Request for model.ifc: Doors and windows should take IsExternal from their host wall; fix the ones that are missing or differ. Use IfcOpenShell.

First a look at what the model holds.

```python
import ifcopenshell
import ifcopenshell.util.element

model = ifcopenshell.open("model.ifc")
print(model.schema)
seen = {}
for e in model.by_type("IfcDoor") + model.by_type("IfcWindow"):
    if not e.FillsVoids:
        continue
    host = e.FillsVoids[0].RelatingOpeningElement.VoidsElements[0].RelatingBuildingElement
    own = ifcopenshell.util.element.get_pset(e, f"Pset_{e.is_a()[3:].removesuffix('StandardCase')}Common", "IsExternal")
    wall = ifcopenshell.util.element.get_pset(host, "Pset_WallCommon", "IsExternal")
    seen[e.is_a(), own, wall] = seen.get((e.is_a(), own, wall), 0) + 1
for (cls, own, wall), count in sorted(seen.items(), key=str):
    print(count, cls, "IsExternal:", own, "| host wall:", wall)
```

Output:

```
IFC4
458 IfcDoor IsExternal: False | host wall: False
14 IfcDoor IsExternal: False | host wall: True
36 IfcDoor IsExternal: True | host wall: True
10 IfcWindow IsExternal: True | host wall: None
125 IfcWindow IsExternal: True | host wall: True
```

```python
import ifcopenshell
import ifcopenshell.api.pset
import ifcopenshell.util.element

model = ifcopenshell.open("model.ifc")

count = 0
for ifc_class, pset_name in (("IfcDoor", "Pset_DoorCommon"), ("IfcWindow", "Pset_WindowCommon")):
    for e in model.by_type(ifc_class):
        if not e.FillsVoids:
            continue
        host = e.FillsVoids[0].RelatingOpeningElement.VoidsElements[0].RelatingBuildingElement
        external = ifcopenshell.util.element.get_pset(host, "Pset_WallCommon", "IsExternal")
        if external is None or ifcopenshell.util.element.get_pset(e, pset_name, "IsExternal") == external:
            continue
        pset = ifcopenshell.api.pset.add_pset(model, product=e, name=pset_name)
        ifcopenshell.api.pset.edit_pset(model, pset=pset, properties={"IsExternal": external})
        count += 1

print(count, "updated")

model.write("model_rev.ifc")
```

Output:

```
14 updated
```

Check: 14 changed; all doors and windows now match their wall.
